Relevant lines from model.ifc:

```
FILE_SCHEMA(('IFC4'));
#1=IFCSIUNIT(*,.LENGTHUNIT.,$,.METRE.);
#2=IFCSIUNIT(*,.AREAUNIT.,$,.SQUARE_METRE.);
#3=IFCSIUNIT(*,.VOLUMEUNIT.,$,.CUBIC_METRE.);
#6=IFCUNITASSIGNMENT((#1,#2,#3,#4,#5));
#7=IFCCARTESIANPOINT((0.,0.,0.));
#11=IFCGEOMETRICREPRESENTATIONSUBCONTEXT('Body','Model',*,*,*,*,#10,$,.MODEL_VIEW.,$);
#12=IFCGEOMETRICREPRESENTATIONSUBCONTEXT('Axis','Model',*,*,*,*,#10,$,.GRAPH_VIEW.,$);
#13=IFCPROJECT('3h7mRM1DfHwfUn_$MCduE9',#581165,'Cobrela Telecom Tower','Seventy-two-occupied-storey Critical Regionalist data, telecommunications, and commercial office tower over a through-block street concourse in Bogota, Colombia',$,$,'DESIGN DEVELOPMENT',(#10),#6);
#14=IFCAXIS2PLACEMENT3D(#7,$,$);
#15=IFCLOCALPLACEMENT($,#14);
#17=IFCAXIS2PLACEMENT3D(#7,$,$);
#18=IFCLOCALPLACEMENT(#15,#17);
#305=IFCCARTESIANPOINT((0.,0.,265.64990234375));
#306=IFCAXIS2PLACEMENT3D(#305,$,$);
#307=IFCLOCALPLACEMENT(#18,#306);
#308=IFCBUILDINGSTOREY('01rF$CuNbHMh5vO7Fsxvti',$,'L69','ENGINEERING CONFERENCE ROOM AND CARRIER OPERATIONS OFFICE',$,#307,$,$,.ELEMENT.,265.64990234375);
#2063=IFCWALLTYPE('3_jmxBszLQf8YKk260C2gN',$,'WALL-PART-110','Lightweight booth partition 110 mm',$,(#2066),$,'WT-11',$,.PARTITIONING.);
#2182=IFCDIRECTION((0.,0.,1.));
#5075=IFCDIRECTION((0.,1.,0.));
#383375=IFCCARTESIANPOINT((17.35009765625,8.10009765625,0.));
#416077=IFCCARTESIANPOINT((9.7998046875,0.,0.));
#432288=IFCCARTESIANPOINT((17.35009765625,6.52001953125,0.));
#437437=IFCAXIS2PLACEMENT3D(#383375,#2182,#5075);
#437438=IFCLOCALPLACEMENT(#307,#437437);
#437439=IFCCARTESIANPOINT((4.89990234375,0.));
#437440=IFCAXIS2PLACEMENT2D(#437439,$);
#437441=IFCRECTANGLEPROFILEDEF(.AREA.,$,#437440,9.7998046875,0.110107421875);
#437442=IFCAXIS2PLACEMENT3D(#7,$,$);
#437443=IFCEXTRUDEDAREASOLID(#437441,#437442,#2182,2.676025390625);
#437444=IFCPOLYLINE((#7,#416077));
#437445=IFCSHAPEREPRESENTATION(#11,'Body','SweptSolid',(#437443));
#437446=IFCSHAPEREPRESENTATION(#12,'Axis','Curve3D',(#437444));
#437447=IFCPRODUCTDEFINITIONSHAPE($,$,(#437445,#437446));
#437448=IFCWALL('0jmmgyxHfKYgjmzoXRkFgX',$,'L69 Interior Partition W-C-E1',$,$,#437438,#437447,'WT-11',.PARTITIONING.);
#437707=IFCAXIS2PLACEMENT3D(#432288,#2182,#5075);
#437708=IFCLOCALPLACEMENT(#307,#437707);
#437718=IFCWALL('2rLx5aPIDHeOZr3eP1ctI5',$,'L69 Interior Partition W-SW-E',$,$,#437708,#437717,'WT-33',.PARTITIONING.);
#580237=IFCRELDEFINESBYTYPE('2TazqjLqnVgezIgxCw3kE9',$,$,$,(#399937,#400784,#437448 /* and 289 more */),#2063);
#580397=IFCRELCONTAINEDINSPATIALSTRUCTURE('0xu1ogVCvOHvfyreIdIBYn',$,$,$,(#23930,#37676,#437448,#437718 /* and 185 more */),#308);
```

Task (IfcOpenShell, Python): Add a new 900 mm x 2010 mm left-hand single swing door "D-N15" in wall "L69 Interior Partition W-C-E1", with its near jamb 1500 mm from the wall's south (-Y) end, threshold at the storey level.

```python
import numpy as np
import ifcopenshell
import ifcopenshell.api.feature
import ifcopenshell.api.geometry
import ifcopenshell.api.root
import ifcopenshell.api.spatial
import ifcopenshell.geom
import ifcopenshell.util.element
import ifcopenshell.util.placement
import ifcopenshell.util.representation
import ifcopenshell.util.shape
import ifcopenshell.util.unit

model = ifcopenshell.open("model.ifc")
unit_scale = ifcopenshell.util.unit.calculate_unit_scale(model)
settings = ifcopenshell.geom.settings()


def volume(element):
    """Net volume in cubic metres, openings subtracted."""
    shape = ifcopenshell.geom.create_shape(settings, element)
    return ifcopenshell.util.shape.get_volume(shape.geometry)


wall = model.by_guid("0jmmgyxHfKYgjmzoXRkFgX")
storey = ifcopenshell.util.element.get_container(wall, ifc_class="IfcBuildingStorey")
context = ifcopenshell.util.representation.get_context(model, "Model", "Body", "MODEL_VIEW")
before = volume(wall)

width, height, from_end, sill = 0.9, 2.01, 1.5, 0.0  # metres

# The wall runs along its own X axis, and the end named is its -X end.
wall_shape = ifcopenshell.geom.create_shape(settings, wall)
x, y, z = ifcopenshell.util.shape.get_vertices(wall_shape.geometry).T
start = x.min() + from_end
face, thickness = float(y.min()), float(y.max() - y.min())
wall_matrix = ifcopenshell.util.placement.get_local_placement(wall.ObjectPlacement)
level = ifcopenshell.util.placement.get_local_placement(storey.ObjectPlacement)[2, 3]


def in_wall(x, y):
    """Placement at x, y metres in the wall's axes, at sill height."""
    matrix = wall_matrix.copy()
    matrix[:, 3] = wall_matrix @ np.array([x / unit_scale, y / unit_scale, 0.0, 1.0])
    matrix[2, 3] = level + sill / unit_scale
    return matrix


# Opening: a box that overshoots both wall faces by 50 mm.
opening = ifcopenshell.api.root.create_entity(model, ifc_class="IfcOpeningElement", predefined_type="OPENING")
box = ifcopenshell.api.geometry.add_wall_representation(
    model, context=context, length=width, height=height, thickness=thickness + 0.1
)
ifcopenshell.api.geometry.assign_representation(model, product=opening, representation=box)
ifcopenshell.api.geometry.edit_object_placement(model, product=opening, matrix=in_wall(start, face - 0.05), is_si=False)
ifcopenshell.api.feature.add_feature(model, feature=opening, element=wall)

door = ifcopenshell.api.root.create_entity(model, ifc_class="IfcDoor", name="D-N15", predefined_type="DOOR")
door.OverallWidth, door.OverallHeight = width / unit_scale, height / unit_scale
door.OperationType = "SINGLE_SWING_LEFT"
body = ifcopenshell.api.geometry.add_door_representation(
    model,
    context=context,
    overall_width=door.OverallWidth,
    overall_height=door.OverallHeight,
    operation_type="SINGLE_SWING_LEFT",
    lining_properties={"LiningDepth": thickness / unit_scale, "ThresholdDepth": thickness / unit_scale},
)
ifcopenshell.api.geometry.assign_representation(model, product=door, representation=body)
ifcopenshell.api.spatial.assign_container(model, products=[door], relating_structure=storey)
ifcopenshell.api.feature.add_filling(model, opening=opening, element=door)

# The lining spans the wall, so the door starts at the wall face.
ifcopenshell.api.geometry.edit_object_placement(model, product=door, matrix=in_wall(start, face), is_si=False)

after = volume(wall)

print(f"wall volume {before:.3f} -> {after:.3f} m3")

model.write("model_rev.ifc")
```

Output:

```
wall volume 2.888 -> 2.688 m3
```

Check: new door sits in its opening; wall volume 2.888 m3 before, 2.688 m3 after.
